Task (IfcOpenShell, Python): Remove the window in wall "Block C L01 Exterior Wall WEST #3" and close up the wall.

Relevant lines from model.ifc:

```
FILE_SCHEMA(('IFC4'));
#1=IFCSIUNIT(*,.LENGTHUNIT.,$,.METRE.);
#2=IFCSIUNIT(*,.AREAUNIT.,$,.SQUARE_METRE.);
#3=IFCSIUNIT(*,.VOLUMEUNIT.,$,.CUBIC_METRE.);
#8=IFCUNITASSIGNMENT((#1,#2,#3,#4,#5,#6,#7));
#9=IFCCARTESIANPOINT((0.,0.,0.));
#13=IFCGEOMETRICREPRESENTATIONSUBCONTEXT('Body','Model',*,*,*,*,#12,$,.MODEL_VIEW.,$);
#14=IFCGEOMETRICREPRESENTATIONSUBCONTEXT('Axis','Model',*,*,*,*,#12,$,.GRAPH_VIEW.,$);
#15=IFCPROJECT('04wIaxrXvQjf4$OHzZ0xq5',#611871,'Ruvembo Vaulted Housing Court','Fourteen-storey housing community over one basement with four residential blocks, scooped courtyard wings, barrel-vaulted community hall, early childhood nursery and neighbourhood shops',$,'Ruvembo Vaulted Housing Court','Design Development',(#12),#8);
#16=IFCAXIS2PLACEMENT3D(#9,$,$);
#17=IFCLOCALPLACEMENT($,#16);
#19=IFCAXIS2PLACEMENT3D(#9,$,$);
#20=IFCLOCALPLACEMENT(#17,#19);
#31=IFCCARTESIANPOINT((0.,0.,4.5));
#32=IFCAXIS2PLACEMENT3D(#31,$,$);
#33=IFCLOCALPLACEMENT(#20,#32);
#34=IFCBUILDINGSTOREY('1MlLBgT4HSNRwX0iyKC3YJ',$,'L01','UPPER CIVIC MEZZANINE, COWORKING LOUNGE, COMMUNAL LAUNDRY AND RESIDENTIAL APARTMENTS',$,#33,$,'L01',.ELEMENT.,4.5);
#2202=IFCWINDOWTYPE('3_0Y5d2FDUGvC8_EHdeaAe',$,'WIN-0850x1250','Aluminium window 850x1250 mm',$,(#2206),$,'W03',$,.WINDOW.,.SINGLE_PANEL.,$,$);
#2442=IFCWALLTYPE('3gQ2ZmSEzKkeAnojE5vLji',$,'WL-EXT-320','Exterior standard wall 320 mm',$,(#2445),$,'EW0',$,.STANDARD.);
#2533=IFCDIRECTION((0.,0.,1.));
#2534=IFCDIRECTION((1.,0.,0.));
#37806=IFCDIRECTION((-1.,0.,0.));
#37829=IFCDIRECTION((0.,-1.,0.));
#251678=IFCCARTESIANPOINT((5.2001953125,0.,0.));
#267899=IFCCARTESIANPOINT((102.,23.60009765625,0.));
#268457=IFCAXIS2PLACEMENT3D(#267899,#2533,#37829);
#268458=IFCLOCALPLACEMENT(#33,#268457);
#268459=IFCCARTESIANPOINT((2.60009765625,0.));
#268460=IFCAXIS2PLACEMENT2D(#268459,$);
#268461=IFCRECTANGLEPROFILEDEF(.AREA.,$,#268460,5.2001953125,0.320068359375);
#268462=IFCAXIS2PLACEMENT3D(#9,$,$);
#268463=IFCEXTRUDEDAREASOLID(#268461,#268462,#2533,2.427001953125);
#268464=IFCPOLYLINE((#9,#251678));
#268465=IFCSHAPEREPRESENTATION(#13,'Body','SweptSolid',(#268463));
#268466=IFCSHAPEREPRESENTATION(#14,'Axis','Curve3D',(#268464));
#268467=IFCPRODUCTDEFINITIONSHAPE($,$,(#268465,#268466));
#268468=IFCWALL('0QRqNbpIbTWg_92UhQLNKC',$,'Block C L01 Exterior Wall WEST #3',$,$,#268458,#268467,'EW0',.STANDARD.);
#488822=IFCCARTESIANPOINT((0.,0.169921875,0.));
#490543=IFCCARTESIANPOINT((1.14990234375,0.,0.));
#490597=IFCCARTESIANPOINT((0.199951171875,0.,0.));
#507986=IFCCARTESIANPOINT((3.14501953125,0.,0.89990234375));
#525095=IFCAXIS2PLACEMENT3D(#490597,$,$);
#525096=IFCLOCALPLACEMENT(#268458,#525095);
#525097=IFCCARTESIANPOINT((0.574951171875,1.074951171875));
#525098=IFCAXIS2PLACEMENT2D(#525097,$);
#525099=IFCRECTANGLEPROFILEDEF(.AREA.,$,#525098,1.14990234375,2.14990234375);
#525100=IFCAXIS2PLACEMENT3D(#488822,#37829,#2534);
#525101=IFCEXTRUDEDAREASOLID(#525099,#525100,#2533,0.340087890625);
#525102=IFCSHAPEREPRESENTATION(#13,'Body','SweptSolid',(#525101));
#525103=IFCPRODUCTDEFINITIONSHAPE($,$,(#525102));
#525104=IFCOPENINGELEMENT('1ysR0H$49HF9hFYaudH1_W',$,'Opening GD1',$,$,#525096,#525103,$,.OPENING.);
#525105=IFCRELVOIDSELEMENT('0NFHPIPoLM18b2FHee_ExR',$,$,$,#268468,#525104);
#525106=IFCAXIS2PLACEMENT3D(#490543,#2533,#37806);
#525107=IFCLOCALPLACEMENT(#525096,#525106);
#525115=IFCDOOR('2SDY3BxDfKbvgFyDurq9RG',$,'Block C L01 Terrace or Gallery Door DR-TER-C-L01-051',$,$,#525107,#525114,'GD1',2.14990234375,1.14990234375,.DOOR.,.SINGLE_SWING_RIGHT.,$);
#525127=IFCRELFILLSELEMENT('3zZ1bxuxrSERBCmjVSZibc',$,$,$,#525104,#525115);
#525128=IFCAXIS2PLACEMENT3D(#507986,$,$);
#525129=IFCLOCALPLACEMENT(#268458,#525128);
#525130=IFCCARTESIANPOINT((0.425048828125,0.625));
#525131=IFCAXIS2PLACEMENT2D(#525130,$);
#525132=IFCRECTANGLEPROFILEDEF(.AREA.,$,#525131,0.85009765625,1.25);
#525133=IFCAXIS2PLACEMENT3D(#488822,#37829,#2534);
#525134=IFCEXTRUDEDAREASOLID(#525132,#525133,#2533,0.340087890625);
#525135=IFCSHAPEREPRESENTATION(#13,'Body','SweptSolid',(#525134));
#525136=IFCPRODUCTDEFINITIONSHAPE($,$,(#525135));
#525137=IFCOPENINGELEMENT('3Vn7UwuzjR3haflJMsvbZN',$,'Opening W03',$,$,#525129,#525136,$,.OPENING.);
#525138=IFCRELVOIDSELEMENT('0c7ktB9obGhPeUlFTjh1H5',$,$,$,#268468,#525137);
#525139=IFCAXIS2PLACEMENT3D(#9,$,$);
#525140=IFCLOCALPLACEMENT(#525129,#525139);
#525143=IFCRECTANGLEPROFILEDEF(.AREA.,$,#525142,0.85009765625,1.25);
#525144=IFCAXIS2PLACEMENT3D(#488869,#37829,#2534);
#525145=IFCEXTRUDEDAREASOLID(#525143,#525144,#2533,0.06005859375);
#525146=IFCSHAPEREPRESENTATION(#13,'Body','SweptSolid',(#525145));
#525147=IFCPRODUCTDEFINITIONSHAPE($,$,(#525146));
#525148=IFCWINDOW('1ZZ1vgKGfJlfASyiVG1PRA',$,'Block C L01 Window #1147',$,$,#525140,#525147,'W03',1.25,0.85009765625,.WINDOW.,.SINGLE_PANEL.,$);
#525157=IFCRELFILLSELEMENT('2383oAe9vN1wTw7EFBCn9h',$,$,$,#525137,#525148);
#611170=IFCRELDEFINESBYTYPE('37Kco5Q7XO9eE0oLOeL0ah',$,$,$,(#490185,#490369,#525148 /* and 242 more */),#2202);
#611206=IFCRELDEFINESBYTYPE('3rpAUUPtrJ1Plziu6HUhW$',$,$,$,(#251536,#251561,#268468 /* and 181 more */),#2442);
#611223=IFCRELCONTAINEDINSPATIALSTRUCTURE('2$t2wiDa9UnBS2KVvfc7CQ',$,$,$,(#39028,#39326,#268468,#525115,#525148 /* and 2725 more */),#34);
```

```python
import ifcopenshell
import ifcopenshell.api.feature
import ifcopenshell.api.root
import ifcopenshell.geom
import ifcopenshell.util.shape

model = ifcopenshell.open("model.ifc")
settings = ifcopenshell.geom.settings()


def volume(element):
    """Net volume in cubic metres, openings subtracted."""
    shape = ifcopenshell.geom.create_shape(settings, element)
    return ifcopenshell.util.shape.get_volume(shape.geometry)


window = model.by_guid("1ZZ1vgKGfJlfASyiVG1PRA")
opening = window.FillsVoids[0].RelatingOpeningElement
wall = opening.VoidsElements[0].RelatingBuildingElement
before = volume(wall)

ifcopenshell.api.root.remove_product(model, product=window)
ifcopenshell.api.feature.remove_feature(model, feature=opening)

after = volume(wall)

print(f"wall volume {before:.3f} -> {after:.3f} m3")

model.write("model_updated.ifc")
```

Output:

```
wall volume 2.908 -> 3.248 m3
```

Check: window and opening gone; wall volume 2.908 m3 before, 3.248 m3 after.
